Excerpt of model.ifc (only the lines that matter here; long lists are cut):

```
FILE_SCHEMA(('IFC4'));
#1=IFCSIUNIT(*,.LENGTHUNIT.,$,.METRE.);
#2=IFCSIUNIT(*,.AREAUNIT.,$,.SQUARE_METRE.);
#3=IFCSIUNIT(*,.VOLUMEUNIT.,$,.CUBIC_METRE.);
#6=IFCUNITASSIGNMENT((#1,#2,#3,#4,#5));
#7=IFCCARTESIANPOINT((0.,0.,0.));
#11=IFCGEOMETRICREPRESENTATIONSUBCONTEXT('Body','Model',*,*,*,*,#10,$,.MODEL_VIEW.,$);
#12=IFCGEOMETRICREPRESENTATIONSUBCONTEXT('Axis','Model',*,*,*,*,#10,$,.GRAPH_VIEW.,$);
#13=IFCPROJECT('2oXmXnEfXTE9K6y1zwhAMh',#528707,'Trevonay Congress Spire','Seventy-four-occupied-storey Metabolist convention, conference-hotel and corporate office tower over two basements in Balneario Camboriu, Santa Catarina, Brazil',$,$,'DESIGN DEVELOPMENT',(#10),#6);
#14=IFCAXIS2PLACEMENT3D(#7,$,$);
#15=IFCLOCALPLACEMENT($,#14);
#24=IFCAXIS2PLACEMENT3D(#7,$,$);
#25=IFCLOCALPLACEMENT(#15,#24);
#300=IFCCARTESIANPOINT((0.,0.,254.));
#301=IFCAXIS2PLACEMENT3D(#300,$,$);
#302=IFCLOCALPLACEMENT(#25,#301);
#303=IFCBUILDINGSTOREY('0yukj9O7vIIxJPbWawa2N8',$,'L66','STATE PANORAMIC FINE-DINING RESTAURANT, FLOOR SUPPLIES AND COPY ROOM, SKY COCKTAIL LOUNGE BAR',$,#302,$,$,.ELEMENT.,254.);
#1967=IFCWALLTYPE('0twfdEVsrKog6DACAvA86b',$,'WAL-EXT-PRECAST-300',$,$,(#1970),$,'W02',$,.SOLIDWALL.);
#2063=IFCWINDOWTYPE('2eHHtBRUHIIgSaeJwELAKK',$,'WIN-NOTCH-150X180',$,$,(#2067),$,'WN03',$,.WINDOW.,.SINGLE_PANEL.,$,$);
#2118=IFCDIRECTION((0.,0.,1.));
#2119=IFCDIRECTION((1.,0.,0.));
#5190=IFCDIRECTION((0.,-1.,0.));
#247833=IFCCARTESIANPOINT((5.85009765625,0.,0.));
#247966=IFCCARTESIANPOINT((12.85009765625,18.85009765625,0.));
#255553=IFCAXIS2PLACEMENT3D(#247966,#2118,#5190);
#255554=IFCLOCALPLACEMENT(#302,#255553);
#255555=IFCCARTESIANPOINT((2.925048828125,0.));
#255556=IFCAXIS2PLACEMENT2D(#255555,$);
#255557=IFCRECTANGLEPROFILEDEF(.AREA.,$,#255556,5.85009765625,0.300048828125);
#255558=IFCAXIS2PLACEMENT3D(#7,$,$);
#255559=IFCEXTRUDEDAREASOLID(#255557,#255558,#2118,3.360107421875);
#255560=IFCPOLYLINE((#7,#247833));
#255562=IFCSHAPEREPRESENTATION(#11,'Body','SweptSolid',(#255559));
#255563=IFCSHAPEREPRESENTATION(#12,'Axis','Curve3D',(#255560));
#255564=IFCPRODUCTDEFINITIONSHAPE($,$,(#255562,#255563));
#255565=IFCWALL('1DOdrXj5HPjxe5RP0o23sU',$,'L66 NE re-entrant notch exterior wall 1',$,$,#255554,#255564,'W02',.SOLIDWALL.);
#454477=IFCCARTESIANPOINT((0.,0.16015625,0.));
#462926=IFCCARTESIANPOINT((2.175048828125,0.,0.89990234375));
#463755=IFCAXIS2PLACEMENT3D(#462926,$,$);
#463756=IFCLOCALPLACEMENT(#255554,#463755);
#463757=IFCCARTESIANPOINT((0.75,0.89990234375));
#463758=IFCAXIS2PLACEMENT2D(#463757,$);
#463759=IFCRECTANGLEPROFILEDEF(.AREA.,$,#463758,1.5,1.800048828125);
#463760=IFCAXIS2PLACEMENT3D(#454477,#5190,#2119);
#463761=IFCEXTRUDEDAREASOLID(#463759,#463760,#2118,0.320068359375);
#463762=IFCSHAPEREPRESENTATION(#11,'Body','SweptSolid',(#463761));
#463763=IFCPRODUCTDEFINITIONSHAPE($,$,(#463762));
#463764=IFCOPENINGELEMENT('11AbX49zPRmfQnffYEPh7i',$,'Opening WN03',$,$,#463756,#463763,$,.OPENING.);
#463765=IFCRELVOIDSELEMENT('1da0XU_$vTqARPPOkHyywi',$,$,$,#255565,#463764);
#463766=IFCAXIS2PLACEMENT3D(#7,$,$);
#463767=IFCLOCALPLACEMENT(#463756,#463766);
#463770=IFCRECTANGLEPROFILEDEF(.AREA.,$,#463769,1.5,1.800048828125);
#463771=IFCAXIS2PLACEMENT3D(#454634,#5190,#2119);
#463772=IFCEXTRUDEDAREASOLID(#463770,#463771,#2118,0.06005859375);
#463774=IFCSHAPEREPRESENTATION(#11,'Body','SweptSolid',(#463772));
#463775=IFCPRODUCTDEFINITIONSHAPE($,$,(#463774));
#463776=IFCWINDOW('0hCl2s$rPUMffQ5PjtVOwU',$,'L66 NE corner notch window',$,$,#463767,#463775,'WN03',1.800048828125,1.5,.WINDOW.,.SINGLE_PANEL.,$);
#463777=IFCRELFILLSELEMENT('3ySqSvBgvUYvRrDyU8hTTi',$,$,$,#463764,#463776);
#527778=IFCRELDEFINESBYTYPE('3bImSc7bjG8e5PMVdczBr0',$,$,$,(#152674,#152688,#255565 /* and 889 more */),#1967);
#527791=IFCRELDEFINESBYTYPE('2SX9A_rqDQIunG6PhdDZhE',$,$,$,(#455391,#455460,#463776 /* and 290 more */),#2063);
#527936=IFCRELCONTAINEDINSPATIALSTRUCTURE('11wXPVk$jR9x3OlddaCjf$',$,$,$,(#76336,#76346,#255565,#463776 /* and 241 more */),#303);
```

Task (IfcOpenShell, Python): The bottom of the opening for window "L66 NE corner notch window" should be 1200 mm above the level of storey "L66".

```python
import numpy as np
import ifcopenshell
import ifcopenshell.api.geometry
import ifcopenshell.geom
import ifcopenshell.util.element
import ifcopenshell.util.placement
import ifcopenshell.util.shape
import ifcopenshell.util.unit

model = ifcopenshell.open("model.ifc")
unit_scale = ifcopenshell.util.unit.calculate_unit_scale(model)

window = model.by_guid("0hCl2s$rPUMffQ5PjtVOwU")
opening = window.FillsVoids[0].RelatingOpeningElement
storey = ifcopenshell.util.element.get_container(window, ifc_class="IfcBuildingStorey")
level = ifcopenshell.util.placement.get_local_placement(storey.ObjectPlacement)[2, 3]

# The opening's origin need not be at the sill, so measure its lowest point.
shape = ifcopenshell.geom.create_shape(ifcopenshell.geom.settings(), opening)
bottom = ifcopenshell.util.shape.get_shape_bottom_elevation(shape, shape.geometry) / unit_scale
dz = level + 1.2 - bottom

shift = np.array([0.0, 0.0, dz])
# The window is placed relative to its opening, so it follows when the opening moves.
matrix = ifcopenshell.util.placement.get_local_placement(opening.ObjectPlacement)
matrix[:3, 3] += shift
ifcopenshell.api.geometry.edit_object_placement(
    model, product=opening, matrix=matrix, is_si=False, should_transform_children=True
)

print(f"moved by {dz * unit_scale:+.3f} m")

model.write("model_rev.ifc")
```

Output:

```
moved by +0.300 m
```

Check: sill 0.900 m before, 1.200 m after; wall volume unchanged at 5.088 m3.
